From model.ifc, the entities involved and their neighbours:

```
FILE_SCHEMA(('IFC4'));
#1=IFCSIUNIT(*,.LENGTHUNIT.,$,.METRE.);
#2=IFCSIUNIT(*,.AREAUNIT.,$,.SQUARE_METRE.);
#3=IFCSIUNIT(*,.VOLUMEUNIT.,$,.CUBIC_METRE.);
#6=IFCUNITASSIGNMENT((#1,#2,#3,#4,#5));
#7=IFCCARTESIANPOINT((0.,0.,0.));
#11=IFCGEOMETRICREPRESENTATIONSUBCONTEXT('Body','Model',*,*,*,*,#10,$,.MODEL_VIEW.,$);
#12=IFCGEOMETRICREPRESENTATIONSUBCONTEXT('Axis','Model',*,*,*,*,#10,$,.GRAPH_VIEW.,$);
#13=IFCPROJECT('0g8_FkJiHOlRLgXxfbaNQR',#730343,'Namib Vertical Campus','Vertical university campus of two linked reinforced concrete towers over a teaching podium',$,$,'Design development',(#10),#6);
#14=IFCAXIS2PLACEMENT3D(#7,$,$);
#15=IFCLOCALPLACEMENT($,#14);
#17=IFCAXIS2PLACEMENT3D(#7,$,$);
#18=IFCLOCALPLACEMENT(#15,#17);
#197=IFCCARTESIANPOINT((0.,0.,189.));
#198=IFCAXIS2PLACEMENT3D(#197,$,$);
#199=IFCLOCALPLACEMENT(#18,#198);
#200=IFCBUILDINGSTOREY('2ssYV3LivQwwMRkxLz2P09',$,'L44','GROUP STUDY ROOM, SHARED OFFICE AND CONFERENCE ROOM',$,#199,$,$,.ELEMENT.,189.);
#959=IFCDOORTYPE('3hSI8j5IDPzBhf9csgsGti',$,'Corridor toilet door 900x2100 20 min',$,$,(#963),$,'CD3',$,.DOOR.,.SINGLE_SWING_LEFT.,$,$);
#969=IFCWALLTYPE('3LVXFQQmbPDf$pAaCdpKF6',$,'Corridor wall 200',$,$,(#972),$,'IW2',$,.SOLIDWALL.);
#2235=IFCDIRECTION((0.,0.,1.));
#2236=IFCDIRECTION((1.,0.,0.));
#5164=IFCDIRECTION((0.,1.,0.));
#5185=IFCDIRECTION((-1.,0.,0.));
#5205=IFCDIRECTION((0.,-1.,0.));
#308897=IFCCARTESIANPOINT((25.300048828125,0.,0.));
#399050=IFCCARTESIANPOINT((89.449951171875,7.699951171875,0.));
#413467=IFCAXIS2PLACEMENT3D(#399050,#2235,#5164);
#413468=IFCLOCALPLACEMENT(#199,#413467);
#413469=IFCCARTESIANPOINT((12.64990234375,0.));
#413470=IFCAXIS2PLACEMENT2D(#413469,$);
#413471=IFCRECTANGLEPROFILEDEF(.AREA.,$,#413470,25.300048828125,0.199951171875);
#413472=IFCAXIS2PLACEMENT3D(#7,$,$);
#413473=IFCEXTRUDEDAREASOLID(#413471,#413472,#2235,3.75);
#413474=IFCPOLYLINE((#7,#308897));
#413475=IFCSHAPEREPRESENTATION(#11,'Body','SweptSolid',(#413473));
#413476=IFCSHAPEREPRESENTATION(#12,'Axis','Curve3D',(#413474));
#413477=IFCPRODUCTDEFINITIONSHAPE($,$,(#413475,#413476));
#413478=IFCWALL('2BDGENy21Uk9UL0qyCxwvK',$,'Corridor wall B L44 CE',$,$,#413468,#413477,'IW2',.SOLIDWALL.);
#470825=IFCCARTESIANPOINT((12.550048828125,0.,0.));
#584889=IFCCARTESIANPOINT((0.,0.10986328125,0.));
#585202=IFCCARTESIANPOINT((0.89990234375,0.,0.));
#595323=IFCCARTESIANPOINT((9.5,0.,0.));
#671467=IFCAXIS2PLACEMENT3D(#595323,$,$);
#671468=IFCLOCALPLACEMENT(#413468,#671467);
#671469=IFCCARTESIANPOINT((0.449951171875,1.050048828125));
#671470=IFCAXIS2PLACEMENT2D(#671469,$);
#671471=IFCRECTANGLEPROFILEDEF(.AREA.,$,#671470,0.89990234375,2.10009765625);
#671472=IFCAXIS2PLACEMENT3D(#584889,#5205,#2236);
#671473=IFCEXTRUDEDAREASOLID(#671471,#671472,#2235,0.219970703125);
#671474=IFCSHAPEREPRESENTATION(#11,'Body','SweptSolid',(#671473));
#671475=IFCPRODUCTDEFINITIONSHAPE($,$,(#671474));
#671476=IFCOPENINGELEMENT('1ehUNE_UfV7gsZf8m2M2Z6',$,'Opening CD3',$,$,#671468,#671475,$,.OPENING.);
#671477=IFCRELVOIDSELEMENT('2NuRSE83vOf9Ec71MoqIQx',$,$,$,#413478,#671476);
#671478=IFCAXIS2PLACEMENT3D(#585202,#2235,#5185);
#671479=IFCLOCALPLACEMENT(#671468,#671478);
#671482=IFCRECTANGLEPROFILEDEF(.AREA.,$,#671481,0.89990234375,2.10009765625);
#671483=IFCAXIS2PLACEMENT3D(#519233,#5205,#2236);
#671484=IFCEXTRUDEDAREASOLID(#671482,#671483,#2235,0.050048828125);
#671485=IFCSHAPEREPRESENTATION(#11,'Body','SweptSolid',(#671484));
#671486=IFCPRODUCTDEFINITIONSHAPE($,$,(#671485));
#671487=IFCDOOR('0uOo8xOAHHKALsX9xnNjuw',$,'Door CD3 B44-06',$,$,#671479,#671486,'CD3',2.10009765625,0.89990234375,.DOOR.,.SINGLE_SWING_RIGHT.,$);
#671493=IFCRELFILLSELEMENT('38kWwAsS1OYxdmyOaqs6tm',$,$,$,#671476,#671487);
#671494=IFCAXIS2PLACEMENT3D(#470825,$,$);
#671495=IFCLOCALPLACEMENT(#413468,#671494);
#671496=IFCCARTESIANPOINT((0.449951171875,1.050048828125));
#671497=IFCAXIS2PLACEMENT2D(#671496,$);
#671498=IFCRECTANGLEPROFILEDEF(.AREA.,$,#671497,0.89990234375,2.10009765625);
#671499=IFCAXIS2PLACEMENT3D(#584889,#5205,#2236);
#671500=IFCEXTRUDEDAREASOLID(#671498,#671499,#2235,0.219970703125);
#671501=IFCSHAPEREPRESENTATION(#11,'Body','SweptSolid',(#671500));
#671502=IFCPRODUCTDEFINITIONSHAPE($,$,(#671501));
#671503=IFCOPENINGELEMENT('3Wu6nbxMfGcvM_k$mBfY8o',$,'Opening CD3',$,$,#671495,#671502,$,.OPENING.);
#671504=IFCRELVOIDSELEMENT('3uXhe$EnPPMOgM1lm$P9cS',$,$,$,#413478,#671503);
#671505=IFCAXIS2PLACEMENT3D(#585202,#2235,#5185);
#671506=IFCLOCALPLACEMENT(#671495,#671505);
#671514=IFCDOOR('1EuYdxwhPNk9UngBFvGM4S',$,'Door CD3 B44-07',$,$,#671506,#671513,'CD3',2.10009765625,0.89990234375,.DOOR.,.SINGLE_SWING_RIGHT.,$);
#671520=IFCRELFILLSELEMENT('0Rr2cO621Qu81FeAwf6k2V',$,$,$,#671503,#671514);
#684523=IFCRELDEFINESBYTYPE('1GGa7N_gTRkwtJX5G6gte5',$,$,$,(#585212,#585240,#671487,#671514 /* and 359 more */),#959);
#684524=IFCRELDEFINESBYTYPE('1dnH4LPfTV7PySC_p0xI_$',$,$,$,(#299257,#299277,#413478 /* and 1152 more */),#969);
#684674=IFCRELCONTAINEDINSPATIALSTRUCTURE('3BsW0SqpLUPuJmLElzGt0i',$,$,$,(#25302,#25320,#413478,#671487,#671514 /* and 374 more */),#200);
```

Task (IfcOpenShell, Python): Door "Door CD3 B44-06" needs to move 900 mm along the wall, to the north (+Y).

```python
import ifcopenshell
import ifcopenshell.api.geometry
import ifcopenshell.util.placement

model = ifcopenshell.open("model.ifc")

door = model.by_guid("0uOo8xOAHHKALsX9xnNjuw")
opening = door.FillsVoids[0].RelatingOpeningElement
wall = opening.VoidsElements[0].RelatingBuildingElement

wall_matrix = ifcopenshell.util.placement.get_local_placement(wall.ObjectPlacement)
shift = wall_matrix[:3, 0] * 0.9
before = ifcopenshell.util.placement.get_local_placement(door.ObjectPlacement)[:3, 3].copy()

# The door is placed relative to its opening, so it follows when the opening moves.
matrix = ifcopenshell.util.placement.get_local_placement(opening.ObjectPlacement)
matrix[:3, 3] += shift
ifcopenshell.api.geometry.edit_object_placement(
    model, product=opening, matrix=matrix, is_si=False, should_transform_children=True
)

after = ifcopenshell.util.placement.get_local_placement(door.ObjectPlacement)[:3, 3]
print("door moved by", (after - before).round(3) + 0.0)

model.write("model_edited.ifc")
```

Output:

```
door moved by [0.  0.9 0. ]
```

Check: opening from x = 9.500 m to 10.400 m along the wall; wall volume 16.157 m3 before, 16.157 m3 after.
